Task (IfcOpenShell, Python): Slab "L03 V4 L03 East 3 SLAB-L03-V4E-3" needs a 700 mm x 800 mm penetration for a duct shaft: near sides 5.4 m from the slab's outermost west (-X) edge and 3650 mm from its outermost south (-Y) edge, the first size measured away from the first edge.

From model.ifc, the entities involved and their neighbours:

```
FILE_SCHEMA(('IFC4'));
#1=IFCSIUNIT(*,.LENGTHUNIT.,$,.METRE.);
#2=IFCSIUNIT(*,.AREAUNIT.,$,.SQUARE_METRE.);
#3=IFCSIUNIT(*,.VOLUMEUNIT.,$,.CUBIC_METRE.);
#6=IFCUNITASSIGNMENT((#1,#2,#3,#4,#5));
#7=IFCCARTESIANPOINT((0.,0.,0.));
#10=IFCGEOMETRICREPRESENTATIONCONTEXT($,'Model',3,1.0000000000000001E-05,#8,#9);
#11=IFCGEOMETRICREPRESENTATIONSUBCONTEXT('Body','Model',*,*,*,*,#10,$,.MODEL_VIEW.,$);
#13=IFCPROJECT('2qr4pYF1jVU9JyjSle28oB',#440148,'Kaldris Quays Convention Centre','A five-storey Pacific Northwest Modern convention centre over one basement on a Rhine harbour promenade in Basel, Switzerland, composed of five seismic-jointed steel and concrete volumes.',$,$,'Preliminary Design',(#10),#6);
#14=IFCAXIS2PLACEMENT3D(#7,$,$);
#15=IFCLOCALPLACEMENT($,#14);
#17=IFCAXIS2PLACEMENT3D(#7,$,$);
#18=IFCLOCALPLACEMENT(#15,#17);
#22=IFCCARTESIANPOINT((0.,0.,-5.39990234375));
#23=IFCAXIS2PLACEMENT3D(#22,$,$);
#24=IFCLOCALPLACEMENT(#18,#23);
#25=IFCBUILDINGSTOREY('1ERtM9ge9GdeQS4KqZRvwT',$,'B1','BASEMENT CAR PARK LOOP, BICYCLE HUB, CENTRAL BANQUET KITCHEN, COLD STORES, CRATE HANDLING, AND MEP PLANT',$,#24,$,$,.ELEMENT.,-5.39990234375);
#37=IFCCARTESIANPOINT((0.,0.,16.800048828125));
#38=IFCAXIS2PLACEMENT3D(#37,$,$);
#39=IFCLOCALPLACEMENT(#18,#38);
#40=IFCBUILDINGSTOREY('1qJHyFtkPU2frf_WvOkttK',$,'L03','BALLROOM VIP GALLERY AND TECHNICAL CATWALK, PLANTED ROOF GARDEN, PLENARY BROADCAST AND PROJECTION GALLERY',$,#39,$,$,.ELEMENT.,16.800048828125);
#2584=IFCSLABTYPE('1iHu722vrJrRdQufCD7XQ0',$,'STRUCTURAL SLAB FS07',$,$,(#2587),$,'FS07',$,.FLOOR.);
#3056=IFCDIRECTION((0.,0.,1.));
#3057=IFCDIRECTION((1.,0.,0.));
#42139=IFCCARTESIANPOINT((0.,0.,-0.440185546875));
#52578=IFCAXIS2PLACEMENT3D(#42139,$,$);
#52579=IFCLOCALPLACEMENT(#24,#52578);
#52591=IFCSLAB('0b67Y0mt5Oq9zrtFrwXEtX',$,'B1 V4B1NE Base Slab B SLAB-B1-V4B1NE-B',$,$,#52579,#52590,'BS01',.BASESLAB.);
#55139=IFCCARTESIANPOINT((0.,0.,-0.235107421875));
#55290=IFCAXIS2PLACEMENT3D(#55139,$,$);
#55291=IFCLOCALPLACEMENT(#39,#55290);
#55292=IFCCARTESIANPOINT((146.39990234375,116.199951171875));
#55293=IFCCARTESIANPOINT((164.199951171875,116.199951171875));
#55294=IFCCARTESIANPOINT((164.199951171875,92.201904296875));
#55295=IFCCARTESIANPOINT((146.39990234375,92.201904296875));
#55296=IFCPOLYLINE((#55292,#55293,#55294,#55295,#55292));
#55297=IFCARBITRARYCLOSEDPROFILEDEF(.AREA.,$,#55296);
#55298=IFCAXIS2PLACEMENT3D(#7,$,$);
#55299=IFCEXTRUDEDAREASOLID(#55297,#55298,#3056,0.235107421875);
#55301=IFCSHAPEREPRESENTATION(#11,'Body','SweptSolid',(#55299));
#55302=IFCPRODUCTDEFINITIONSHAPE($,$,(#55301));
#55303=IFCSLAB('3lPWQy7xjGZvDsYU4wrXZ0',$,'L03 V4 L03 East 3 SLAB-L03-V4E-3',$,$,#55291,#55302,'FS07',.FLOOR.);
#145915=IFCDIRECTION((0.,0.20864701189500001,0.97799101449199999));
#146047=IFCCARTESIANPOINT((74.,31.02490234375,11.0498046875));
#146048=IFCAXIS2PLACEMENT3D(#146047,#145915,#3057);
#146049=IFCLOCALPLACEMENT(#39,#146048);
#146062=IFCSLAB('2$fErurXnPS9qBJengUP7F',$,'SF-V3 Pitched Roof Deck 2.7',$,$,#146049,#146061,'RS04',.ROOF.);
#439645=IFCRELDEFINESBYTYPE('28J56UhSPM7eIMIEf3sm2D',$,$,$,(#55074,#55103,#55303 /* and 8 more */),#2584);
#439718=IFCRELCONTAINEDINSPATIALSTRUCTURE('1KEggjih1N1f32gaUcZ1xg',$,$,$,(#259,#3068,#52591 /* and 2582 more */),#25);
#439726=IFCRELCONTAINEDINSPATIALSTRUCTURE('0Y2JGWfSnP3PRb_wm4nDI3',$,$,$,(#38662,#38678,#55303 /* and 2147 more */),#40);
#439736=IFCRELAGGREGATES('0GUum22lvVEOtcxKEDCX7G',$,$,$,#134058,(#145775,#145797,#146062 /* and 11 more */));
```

```python
import numpy as np
import ifcopenshell
import ifcopenshell.api.feature
import ifcopenshell.api.geometry
import ifcopenshell.api.root
import ifcopenshell.geom
import ifcopenshell.util.placement
import ifcopenshell.util.representation
import ifcopenshell.util.shape
import ifcopenshell.util.unit

model = ifcopenshell.open("model.ifc")
unit_scale = ifcopenshell.util.unit.calculate_unit_scale(model)
settings = ifcopenshell.geom.settings()


def volume(element):
    """Net volume in cubic metres, openings subtracted."""
    shape = ifcopenshell.geom.create_shape(settings, element)
    return ifcopenshell.util.shape.get_volume(shape.geometry)


slab = model.by_id(55303)
before = volume(slab)

# Extent in the slab's own axes, in metres. The edges named are its -X and -Y sides.
slab_shape = ifcopenshell.geom.create_shape(settings, slab)
vertices = ifcopenshell.util.shape.get_vertices(slab_shape.geometry)
x_min, y_min, bottom = vertices.min(axis=0)
top = vertices[:, 2].max()

opening = ifcopenshell.api.root.create_entity(model, ifc_class="IfcOpeningElement", name="Duct shaft opening", predefined_type="OPENING")
context = ifcopenshell.util.representation.get_context(model, "Model", "Body", "MODEL_VIEW")
width, depth = 0.7, 0.8
outline = [(0.0, 0.0), (width, 0.0), (width, depth), (0.0, depth), (0.0, 0.0)]
# Overshoot both faces by 50 mm so the cut is clean.
shape = ifcopenshell.api.geometry.add_slab_representation(
    model, context=context, depth=top - bottom + 0.1, polyline=outline
)
ifcopenshell.api.geometry.assign_representation(model, product=opening, representation=shape)

matrix = ifcopenshell.util.placement.get_local_placement(slab.ObjectPlacement)
matrix[:, 3] = matrix @ np.append(np.array([x_min + 5.4, y_min + 3.65, bottom - 0.05]) / unit_scale, 1.0)
ifcopenshell.api.geometry.edit_object_placement(model, product=opening, matrix=matrix, is_si=False)
ifcopenshell.api.feature.add_feature(model, feature=opening, element=slab)

after = volume(slab)

print(f"slab volume {before:.3f} -> {after:.3f} m3")

model.write("model_rev.ifc")
```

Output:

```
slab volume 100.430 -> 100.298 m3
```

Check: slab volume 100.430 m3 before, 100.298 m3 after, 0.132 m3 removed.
